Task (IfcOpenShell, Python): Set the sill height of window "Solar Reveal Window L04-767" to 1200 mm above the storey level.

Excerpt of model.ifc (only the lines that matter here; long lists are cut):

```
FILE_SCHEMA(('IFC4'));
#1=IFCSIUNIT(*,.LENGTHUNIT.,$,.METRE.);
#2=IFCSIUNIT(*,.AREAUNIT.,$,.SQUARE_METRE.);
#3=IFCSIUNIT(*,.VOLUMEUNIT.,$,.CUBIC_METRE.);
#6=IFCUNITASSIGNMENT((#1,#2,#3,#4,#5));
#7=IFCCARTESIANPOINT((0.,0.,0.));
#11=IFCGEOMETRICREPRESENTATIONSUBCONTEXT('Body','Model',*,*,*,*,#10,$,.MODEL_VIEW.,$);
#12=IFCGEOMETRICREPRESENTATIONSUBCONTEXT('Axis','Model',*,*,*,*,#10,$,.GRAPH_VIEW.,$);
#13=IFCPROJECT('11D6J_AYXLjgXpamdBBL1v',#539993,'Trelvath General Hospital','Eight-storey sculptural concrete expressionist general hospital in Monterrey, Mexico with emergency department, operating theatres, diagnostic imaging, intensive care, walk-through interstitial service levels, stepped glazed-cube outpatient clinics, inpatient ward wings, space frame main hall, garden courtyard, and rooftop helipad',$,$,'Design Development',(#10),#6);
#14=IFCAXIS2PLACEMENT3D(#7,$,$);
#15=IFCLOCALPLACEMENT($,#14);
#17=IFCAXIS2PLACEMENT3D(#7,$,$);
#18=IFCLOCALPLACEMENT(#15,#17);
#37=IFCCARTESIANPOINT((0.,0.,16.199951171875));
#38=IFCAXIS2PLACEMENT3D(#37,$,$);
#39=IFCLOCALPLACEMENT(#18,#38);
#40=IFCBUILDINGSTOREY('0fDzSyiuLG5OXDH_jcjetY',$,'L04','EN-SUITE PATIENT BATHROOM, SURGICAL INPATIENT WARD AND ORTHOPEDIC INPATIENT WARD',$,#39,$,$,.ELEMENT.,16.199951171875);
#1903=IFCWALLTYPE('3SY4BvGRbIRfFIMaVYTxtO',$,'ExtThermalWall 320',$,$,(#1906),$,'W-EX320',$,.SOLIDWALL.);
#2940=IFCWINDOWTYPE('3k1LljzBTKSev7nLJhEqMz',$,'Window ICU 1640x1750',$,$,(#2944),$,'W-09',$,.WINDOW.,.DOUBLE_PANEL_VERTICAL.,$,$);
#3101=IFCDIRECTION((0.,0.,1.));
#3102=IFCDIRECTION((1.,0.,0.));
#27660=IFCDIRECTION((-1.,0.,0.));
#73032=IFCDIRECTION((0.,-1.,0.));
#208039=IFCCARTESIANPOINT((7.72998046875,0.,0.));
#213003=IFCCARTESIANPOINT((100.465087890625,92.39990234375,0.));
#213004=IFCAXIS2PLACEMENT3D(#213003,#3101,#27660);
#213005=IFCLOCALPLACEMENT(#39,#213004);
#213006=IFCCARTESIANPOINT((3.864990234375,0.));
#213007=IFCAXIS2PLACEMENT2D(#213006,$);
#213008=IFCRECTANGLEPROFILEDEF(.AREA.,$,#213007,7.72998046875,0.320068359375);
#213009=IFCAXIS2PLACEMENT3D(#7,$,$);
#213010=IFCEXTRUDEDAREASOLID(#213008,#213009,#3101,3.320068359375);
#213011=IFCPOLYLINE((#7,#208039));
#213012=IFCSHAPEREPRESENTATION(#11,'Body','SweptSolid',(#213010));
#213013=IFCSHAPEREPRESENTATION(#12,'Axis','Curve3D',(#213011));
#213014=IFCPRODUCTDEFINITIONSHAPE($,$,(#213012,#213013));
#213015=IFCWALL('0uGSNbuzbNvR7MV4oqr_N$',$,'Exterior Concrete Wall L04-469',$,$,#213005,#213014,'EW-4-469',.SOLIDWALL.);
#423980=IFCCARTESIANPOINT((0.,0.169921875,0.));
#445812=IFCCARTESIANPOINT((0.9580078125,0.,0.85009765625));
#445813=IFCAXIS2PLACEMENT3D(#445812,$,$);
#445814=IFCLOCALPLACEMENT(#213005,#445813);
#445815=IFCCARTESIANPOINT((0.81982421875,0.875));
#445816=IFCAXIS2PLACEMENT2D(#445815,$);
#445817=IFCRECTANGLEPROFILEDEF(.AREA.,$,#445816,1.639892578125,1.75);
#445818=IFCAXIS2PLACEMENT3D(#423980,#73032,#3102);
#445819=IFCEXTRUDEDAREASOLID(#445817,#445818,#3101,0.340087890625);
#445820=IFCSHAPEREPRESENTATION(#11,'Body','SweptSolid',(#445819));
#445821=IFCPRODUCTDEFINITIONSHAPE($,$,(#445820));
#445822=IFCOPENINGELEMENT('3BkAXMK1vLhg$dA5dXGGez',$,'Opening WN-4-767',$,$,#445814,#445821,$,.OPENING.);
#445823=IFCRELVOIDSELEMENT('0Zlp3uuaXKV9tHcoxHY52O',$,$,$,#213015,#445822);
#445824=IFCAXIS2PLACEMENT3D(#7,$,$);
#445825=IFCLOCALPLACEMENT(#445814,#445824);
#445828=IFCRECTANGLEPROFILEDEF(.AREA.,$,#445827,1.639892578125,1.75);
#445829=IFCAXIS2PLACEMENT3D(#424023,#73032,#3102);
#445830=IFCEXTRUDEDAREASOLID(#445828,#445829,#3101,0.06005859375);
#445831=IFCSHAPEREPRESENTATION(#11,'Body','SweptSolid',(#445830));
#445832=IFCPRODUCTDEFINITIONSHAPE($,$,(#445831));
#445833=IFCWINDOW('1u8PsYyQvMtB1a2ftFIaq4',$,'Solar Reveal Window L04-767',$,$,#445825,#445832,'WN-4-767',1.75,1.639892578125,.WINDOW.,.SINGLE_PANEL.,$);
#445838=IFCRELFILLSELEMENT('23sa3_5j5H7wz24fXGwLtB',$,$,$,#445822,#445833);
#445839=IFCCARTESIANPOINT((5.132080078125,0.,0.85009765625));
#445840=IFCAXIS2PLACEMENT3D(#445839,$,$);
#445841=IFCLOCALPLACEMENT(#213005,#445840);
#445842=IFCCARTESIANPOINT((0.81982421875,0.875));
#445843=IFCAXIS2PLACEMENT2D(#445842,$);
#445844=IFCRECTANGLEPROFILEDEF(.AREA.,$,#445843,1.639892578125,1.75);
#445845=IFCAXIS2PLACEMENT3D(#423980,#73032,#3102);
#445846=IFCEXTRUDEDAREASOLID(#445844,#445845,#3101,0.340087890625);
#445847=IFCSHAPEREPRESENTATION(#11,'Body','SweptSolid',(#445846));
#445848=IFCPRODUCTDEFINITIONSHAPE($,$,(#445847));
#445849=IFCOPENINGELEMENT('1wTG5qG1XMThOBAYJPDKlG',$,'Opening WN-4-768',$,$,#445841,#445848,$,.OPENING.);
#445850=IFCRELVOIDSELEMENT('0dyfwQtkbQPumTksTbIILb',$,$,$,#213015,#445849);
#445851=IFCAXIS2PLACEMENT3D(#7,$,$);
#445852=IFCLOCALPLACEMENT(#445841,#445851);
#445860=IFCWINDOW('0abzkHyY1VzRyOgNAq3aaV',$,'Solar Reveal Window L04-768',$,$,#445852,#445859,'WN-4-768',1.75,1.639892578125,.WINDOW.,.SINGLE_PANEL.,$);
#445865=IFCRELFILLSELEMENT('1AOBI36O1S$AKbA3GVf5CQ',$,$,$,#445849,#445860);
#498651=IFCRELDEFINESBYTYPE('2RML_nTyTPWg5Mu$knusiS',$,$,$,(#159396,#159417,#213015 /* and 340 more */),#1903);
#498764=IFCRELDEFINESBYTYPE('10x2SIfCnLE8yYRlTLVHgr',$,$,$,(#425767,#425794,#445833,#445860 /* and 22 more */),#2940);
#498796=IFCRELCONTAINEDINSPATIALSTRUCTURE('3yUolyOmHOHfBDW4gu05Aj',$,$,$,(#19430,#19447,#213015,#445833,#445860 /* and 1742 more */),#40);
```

```python
import numpy as np
import ifcopenshell
import ifcopenshell.api.geometry
import ifcopenshell.geom
import ifcopenshell.util.element
import ifcopenshell.util.placement
import ifcopenshell.util.shape
import ifcopenshell.util.unit

model = ifcopenshell.open("model.ifc")
unit_scale = ifcopenshell.util.unit.calculate_unit_scale(model)

window = model.by_guid("1u8PsYyQvMtB1a2ftFIaq4")
opening = window.FillsVoids[0].RelatingOpeningElement
storey = ifcopenshell.util.element.get_container(window, ifc_class="IfcBuildingStorey")
level = ifcopenshell.util.placement.get_local_placement(storey.ObjectPlacement)[2, 3]

# The opening's origin need not be at the sill, so measure its lowest point.
shape = ifcopenshell.geom.create_shape(ifcopenshell.geom.settings(), opening)
bottom = ifcopenshell.util.shape.get_shape_bottom_elevation(shape, shape.geometry) / unit_scale
dz = level + 1.2 / unit_scale - bottom

shift = np.array([0.0, 0.0, dz])
# The window is placed relative to its opening, so it follows when the opening moves.
matrix = ifcopenshell.util.placement.get_local_placement(opening.ObjectPlacement)
matrix[:3, 3] += shift
ifcopenshell.api.geometry.edit_object_placement(
    model, product=opening, matrix=matrix, is_si=False, should_transform_children=True
)

print(f"moved by {dz * unit_scale:+.3f} m")

model.write("model_updated.ifc")
```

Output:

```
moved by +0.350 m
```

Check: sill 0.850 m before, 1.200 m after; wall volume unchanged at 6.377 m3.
